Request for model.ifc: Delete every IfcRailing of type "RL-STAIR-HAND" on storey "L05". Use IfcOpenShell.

First a look at what the model holds.

```python
import ifcopenshell
import ifcopenshell.util.element

model = ifcopenshell.open("model.ifc")
print(model.schema)
storey = next(s for s in model.by_type("IfcBuildingStorey") if s.Name == "L05")
railings = [e for e in ifcopenshell.util.element.get_decomposition(storey) if e.is_a("IfcRailing")]
seen = {}
for e in railings:
    element_type = ifcopenshell.util.element.get_type(e)
    name = element_type.Name if element_type not in (None, e) else None
    seen[name] = seen.get(name, 0) + 1
for name, count in sorted(seen.items(), key=str):
    print(count, "x", name)
```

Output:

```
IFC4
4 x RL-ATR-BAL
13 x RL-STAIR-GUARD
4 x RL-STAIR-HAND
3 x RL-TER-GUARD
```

```python
import ifcopenshell
import ifcopenshell.api.root
import ifcopenshell.util.element

model = ifcopenshell.open("model.ifc")

storey = next(s for s in model.by_type("IfcBuildingStorey") if s.Name == "L05")
railings = [e for e in ifcopenshell.util.element.get_decomposition(storey) if e.is_a("IfcRailing")]
targets = [e for e in railings if (t := ifcopenshell.util.element.get_type(e)) not in (None, e) and t.Name == "RL-STAIR-HAND"]

for e in targets:
    ifcopenshell.api.root.remove_product(model, product=e)
print(len(targets), "removed")

model.write("model_rev.ifc")
```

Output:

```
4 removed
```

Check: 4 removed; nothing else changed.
